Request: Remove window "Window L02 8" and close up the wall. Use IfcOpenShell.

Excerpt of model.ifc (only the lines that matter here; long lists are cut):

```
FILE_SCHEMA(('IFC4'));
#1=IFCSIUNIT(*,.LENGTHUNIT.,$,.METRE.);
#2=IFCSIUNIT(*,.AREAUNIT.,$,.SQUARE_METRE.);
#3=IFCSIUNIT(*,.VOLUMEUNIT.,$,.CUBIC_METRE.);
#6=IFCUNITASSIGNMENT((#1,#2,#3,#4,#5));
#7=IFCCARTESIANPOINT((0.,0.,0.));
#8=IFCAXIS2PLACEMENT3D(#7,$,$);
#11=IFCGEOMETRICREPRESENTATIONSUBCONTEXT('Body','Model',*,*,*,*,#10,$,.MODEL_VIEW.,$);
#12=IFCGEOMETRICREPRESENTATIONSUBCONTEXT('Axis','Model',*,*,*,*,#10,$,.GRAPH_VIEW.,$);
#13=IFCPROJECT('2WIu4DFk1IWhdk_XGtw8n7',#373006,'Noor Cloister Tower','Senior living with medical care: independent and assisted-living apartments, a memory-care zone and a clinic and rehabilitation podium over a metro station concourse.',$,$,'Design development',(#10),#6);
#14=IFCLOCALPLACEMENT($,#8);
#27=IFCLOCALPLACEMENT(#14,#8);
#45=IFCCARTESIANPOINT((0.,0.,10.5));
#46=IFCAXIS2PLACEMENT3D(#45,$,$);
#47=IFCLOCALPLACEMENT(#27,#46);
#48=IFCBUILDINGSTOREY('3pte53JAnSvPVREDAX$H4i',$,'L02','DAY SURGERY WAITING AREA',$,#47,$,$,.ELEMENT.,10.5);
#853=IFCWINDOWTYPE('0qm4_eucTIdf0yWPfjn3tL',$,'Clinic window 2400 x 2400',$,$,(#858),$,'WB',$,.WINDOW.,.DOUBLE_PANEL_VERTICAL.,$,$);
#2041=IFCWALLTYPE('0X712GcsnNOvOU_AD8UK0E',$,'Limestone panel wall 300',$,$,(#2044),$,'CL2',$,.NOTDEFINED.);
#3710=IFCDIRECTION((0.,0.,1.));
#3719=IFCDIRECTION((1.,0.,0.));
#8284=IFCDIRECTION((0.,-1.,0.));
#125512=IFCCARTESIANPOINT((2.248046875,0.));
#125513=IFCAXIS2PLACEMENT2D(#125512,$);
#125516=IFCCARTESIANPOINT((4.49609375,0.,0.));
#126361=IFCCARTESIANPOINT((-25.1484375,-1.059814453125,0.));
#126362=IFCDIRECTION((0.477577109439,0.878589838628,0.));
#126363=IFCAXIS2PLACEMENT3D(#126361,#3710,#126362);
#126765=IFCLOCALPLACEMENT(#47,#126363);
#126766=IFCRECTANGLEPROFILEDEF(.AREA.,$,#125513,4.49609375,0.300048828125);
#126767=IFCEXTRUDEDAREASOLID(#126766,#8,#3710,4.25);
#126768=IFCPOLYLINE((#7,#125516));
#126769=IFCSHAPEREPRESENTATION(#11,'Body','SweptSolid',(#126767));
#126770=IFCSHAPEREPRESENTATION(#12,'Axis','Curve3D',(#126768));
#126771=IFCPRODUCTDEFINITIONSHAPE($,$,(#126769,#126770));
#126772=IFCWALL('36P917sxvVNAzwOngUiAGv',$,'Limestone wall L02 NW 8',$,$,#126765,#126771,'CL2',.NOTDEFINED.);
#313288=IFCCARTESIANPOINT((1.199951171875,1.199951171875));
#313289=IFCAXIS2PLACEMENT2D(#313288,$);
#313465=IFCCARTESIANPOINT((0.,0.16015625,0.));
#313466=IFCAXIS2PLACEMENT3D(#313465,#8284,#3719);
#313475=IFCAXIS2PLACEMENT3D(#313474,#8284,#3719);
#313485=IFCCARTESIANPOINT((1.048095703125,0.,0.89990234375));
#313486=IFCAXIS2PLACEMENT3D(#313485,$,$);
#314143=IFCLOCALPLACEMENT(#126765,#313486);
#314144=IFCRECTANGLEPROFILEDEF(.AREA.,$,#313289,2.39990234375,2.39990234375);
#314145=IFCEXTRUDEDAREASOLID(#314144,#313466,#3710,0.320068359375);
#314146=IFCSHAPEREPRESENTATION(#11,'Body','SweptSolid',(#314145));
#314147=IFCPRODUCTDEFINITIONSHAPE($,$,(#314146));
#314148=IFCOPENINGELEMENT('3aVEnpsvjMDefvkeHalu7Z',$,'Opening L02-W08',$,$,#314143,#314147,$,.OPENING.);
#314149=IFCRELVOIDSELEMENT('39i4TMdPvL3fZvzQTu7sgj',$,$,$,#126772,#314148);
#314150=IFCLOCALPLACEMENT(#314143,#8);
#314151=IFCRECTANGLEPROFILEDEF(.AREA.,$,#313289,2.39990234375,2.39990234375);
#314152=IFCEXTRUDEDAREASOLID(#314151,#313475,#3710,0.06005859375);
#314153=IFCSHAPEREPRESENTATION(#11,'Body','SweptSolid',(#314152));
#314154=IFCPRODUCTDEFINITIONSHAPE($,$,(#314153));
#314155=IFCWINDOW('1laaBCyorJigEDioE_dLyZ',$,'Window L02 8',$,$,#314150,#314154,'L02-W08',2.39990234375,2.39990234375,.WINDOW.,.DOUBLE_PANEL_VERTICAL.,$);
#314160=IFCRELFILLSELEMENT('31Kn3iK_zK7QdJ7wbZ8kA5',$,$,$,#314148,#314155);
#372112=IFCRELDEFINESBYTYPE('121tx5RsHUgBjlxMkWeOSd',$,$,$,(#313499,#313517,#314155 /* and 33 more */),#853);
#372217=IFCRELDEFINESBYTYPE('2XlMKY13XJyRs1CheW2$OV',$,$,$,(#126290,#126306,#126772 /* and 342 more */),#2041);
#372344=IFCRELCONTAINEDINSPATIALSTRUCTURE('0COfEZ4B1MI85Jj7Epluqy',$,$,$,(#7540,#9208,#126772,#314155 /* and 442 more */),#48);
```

```python
import ifcopenshell
import ifcopenshell.api.feature
import ifcopenshell.api.root
import ifcopenshell.geom
import ifcopenshell.util.shape

model = ifcopenshell.open("model.ifc")
settings = ifcopenshell.geom.settings()


def volume(element):
    """Net volume in cubic metres, openings subtracted."""
    shape = ifcopenshell.geom.create_shape(settings, element)
    return ifcopenshell.util.shape.get_volume(shape.geometry)


window = model.by_guid("1laaBCyorJigEDioE_dLyZ")
opening = window.FillsVoids[0].RelatingOpeningElement
wall = opening.VoidsElements[0].RelatingBuildingElement
before = volume(wall)

ifcopenshell.api.root.remove_product(model, product=window)
ifcopenshell.api.feature.remove_feature(model, feature=opening)

after = volume(wall)

print(f"wall volume {before:.3f} -> {after:.3f} m3")

model.write("model-out.ifc")
```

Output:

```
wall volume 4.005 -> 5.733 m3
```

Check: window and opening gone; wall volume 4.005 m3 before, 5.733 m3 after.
